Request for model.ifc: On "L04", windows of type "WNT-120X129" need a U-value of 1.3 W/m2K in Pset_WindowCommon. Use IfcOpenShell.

First a look at what the model holds.

```python
import ifcopenshell
import ifcopenshell.util.element

model = ifcopenshell.open("model.ifc")
print(model.schema)
storey = next(s for s in model.by_type("IfcBuildingStorey") if s.Name == "L04")
windows = [e for e in ifcopenshell.util.element.get_decomposition(storey) if e.is_a("IfcWindow")]
seen = {}
for e in windows:
    element_type = ifcopenshell.util.element.get_type(e)
    key = (element_type.Name if element_type != e and element_type else None, ifcopenshell.util.element.get_pset(e, "Pset_WindowCommon", "ThermalTransmittance"))
    seen[key] = seen.get(key, 0) + 1
for (name, value), count in sorted(seen.items(), key=str):
    print(count, "x", name, "|", value)
```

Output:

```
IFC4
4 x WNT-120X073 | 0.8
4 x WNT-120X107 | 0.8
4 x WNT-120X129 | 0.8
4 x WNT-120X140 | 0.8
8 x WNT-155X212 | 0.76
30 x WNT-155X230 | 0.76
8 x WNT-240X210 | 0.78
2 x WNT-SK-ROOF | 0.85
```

```python
import ifcopenshell
import ifcopenshell.api.pset
import ifcopenshell.util.element

model = ifcopenshell.open("model.ifc")

storey = next(s for s in model.by_type("IfcBuildingStorey") if s.Name == "L04")
windows = [e for e in ifcopenshell.util.element.get_decomposition(storey) if e.is_a("IfcWindow")]

count = 0
for e in windows:
    element_type = ifcopenshell.util.element.get_type(e)
    if element_type in (None, e) or element_type.Name != "WNT-120X129":
        continue
    # add_pset returns the element's existing set when there is one.
    pset = ifcopenshell.api.pset.add_pset(model, product=e, name="Pset_WindowCommon")
    ifcopenshell.api.pset.edit_pset(model, pset=pset, properties={"ThermalTransmittance": 1.3})
    count += 1

print(count, "windows updated")

model.write("model_updated.ifc")
```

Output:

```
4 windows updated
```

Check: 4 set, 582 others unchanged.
